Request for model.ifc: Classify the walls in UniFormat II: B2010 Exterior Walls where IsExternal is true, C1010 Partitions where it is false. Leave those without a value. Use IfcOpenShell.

First a look at what the model holds.

```python
import ifcopenshell
import ifcopenshell.util.element

model = ifcopenshell.open("model.ifc")
print(model.schema)
print("classifications:", [c.Name for c in model.by_type("IfcClassification")])
values = [ifcopenshell.util.element.get_pset(e, "Pset_WallCommon", "IsExternal") for e in model.by_type("IfcWall")]
for value in (True, False, None):
    print("IsExternal", value, values.count(value))
```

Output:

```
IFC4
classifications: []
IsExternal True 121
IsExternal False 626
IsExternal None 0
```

```python
import ifcopenshell
import ifcopenshell.api.classification
import ifcopenshell.util.element

model = ifcopenshell.open("model.ifc")

system = ifcopenshell.api.classification.add_classification(model, classification="UniFormat II")

walls = model.by_type("IfcWall")
external = {e: ifcopenshell.util.element.get_pset(e, "Pset_WallCommon", "IsExternal") for e in walls}
for flag, code, name in ((True, "B2010", "Exterior Walls"), (False, "C1010", "Partitions")):
    products = [e for e in walls if external[e] is flag]
    ifcopenshell.api.classification.add_reference(
        model, products=products, classification=system, identification=code, name=name
    )
    print(code, len(products))

model.write("model_updated.ifc")
```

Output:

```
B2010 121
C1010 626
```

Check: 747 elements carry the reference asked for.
